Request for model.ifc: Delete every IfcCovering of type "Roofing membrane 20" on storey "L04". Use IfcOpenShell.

First a look at what the model holds.

```python
import ifcopenshell
import ifcopenshell.util.element

model = ifcopenshell.open("model.ifc")
print(model.schema)
storey = next(s for s in model.by_type("IfcBuildingStorey") if s.Name == "L04")
coverings = [e for e in ifcopenshell.util.element.get_decomposition(storey) if e.is_a("IfcCovering")]
seen = {}
for e in coverings:
    element_type = ifcopenshell.util.element.get_type(e)
    name = element_type.Name if element_type not in (None, e) else None
    seen[name] = seen.get(name, 0) + 1
for name, count in sorted(seen.items(), key=str):
    print(count, "x", name)
```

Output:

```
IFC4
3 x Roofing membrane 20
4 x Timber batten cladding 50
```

```python
import ifcopenshell
import ifcopenshell.api.root
import ifcopenshell.util.element

model = ifcopenshell.open("model.ifc")

storey = next(s for s in model.by_type("IfcBuildingStorey") if s.Name == "L04")
coverings = [e for e in ifcopenshell.util.element.get_decomposition(storey) if e.is_a("IfcCovering")]
targets = [e for e in coverings if (t := ifcopenshell.util.element.get_type(e)) not in (None, e) and t.Name == "Roofing membrane 20"]

for e in targets:
    ifcopenshell.api.root.remove_product(model, product=e)
print(len(targets), "removed")

model.write("model-out.ifc")
```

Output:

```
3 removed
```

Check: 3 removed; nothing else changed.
